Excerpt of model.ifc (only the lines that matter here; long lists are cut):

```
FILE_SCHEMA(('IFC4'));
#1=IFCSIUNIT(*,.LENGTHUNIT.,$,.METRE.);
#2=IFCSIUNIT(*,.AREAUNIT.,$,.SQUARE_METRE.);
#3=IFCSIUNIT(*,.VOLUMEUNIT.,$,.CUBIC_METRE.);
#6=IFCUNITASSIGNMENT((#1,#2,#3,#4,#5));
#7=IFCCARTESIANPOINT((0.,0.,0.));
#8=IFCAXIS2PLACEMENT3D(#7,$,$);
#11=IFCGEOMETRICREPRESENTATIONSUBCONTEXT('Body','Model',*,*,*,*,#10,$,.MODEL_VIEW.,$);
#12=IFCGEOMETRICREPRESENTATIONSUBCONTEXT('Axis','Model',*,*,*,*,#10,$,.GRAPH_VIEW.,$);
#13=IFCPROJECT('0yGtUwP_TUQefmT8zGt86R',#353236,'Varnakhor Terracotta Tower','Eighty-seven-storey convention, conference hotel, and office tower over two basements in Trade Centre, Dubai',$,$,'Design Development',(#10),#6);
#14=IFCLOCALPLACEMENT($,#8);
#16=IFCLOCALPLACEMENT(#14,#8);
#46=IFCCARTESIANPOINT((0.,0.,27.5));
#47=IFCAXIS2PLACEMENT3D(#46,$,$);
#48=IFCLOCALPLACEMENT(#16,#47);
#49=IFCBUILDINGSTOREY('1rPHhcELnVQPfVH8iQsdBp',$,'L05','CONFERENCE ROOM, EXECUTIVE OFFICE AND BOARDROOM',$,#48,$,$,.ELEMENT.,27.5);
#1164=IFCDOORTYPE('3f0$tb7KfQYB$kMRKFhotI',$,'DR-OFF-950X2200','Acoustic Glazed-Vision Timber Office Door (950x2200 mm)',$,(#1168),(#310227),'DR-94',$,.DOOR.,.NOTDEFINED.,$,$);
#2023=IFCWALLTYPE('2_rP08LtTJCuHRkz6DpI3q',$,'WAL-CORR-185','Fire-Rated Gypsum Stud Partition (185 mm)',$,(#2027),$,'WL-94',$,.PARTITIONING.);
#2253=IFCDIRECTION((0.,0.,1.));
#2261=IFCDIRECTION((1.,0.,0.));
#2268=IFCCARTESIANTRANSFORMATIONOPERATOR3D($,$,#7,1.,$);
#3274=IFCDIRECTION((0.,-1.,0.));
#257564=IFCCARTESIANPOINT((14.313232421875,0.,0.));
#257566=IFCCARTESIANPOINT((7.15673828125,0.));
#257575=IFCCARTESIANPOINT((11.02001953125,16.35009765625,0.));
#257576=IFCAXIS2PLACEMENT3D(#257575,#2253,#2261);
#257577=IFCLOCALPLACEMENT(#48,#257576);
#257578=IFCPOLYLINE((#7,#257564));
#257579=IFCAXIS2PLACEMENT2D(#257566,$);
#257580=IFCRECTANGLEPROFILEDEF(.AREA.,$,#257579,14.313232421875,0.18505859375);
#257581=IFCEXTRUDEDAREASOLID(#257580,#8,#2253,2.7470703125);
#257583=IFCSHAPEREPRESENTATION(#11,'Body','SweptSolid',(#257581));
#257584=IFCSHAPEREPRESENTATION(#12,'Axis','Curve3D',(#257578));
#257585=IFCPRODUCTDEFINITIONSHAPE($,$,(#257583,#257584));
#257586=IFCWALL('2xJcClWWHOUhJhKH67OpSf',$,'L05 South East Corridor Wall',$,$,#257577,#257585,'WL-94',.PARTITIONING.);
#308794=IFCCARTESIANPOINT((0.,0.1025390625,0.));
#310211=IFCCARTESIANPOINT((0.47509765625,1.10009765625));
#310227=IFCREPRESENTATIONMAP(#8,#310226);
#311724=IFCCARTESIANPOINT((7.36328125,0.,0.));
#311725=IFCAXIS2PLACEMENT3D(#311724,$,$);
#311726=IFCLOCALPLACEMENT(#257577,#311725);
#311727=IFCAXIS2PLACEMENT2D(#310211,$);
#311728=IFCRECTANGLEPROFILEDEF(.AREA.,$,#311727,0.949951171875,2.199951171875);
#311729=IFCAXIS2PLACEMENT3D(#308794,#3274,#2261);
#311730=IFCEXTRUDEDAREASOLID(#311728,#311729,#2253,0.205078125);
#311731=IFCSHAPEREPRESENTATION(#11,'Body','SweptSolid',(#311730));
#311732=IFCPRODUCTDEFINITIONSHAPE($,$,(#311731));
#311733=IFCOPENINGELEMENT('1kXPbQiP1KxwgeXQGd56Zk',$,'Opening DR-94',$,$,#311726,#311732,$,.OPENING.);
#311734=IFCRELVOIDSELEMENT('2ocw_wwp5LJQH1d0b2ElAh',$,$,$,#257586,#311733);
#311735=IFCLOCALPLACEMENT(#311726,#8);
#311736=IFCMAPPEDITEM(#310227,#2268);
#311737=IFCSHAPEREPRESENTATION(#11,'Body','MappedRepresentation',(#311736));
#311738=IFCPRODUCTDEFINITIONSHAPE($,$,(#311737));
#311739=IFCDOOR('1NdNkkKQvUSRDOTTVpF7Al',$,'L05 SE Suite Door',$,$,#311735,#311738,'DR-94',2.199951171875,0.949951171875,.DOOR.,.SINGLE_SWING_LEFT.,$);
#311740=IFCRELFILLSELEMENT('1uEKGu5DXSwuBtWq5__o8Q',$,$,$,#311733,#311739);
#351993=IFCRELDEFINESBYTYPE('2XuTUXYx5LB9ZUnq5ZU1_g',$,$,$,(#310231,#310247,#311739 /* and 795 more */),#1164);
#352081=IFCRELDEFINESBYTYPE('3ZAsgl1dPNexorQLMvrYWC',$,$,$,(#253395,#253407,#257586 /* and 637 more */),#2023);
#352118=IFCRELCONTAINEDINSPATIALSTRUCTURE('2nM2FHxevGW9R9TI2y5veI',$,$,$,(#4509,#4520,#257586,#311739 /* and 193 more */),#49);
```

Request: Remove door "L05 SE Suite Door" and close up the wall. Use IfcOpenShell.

```python
import ifcopenshell
import ifcopenshell.api.feature
import ifcopenshell.api.root
import ifcopenshell.geom
import ifcopenshell.util.shape

model = ifcopenshell.open("model.ifc")
settings = ifcopenshell.geom.settings()


def volume(element):
    """Net volume in cubic metres, openings subtracted."""
    shape = ifcopenshell.geom.create_shape(settings, element)
    return ifcopenshell.util.shape.get_volume(shape.geometry)


door = model.by_guid("1NdNkkKQvUSRDOTTVpF7Al")
opening = door.FillsVoids[0].RelatingOpeningElement
wall = opening.VoidsElements[0].RelatingBuildingElement
before = volume(wall)

ifcopenshell.api.root.remove_product(model, product=door)
ifcopenshell.api.feature.remove_feature(model, feature=opening)

after = volume(wall)

print(f"wall volume {before:.3f} -> {after:.3f} m3")

model.write("model_rev.ifc")
```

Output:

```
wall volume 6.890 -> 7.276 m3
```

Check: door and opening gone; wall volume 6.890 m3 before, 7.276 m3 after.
